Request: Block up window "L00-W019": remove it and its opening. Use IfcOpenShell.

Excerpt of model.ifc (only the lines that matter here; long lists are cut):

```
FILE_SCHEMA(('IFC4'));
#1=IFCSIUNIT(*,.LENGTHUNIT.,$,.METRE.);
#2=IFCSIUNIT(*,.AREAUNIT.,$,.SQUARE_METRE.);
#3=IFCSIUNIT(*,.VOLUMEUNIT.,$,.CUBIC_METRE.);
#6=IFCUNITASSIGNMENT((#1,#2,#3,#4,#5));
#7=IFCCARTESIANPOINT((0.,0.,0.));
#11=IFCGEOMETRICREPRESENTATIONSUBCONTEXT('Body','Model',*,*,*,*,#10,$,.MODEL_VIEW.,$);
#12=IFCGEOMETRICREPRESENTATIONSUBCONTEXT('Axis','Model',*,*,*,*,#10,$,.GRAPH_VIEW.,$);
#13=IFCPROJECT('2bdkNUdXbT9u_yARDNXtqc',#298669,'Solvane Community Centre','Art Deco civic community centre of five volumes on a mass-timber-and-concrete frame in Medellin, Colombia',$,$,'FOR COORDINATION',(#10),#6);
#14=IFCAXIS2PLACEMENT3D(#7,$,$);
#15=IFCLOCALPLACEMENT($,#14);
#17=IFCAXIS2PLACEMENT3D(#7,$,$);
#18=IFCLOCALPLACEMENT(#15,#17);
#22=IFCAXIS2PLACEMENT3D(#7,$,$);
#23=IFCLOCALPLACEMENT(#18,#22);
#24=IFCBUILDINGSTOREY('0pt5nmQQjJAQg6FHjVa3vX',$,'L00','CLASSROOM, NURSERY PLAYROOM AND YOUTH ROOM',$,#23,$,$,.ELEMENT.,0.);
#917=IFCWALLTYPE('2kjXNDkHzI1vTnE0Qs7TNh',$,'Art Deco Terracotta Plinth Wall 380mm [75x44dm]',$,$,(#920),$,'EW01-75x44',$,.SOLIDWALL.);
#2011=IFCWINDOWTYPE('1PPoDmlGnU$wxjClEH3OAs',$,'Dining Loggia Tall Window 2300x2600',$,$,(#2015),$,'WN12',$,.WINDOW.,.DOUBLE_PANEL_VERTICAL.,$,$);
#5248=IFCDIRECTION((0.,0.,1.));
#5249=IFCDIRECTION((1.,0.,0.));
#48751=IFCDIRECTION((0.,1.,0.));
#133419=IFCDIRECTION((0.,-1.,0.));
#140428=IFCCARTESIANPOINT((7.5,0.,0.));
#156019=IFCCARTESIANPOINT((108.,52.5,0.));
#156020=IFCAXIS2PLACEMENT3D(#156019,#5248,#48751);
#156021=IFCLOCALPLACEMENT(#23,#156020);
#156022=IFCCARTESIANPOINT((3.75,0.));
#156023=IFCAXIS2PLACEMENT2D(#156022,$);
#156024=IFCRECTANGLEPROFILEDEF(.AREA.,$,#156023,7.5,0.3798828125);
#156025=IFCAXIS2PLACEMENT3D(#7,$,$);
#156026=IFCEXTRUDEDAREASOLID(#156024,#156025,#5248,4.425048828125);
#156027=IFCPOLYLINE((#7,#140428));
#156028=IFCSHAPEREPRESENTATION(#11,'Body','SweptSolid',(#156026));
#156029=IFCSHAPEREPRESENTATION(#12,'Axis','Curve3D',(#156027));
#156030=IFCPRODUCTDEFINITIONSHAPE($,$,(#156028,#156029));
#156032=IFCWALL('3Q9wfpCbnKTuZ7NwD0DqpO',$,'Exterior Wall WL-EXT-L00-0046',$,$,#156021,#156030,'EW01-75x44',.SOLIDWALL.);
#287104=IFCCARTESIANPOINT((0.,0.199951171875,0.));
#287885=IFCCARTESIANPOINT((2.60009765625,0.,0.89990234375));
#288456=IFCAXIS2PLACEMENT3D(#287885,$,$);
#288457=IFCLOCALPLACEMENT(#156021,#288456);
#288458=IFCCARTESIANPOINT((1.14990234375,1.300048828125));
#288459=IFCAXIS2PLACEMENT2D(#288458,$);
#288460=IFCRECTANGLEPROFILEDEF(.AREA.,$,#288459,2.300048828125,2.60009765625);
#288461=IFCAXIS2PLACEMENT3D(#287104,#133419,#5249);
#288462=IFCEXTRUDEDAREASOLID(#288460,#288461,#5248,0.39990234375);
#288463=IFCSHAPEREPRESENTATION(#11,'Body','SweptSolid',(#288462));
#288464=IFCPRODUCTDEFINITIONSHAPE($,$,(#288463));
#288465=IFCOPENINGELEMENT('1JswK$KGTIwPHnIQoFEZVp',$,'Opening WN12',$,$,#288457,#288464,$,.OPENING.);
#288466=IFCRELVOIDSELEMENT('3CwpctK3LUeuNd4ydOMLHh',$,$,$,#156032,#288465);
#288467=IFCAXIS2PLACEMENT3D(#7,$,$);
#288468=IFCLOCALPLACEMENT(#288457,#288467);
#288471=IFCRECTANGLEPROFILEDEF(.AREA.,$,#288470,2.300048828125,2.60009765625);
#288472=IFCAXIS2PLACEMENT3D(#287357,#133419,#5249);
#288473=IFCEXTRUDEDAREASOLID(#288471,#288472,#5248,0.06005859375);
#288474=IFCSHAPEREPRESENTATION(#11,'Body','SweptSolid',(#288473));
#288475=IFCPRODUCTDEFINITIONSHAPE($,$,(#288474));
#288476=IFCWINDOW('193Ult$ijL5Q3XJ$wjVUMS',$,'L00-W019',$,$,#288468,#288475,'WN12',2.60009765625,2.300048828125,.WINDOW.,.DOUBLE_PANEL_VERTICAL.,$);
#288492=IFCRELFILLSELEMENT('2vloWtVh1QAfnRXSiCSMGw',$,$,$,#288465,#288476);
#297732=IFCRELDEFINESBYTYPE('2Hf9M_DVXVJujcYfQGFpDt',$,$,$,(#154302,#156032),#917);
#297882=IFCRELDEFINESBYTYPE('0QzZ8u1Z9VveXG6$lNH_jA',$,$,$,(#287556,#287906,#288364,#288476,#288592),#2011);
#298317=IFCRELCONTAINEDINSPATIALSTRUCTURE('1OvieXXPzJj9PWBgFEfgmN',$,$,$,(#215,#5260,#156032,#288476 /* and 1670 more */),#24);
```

```python
import ifcopenshell
import ifcopenshell.api.feature
import ifcopenshell.api.root
import ifcopenshell.geom
import ifcopenshell.util.shape

model = ifcopenshell.open("model.ifc")
settings = ifcopenshell.geom.settings()


def volume(element):
    """Net volume in cubic metres, openings subtracted."""
    shape = ifcopenshell.geom.create_shape(settings, element)
    return ifcopenshell.util.shape.get_volume(shape.geometry)


window = model.by_id(288476)
opening = window.FillsVoids[0].RelatingOpeningElement
wall = opening.VoidsElements[0].RelatingBuildingElement
before = volume(wall)

ifcopenshell.api.root.remove_product(model, product=window)
ifcopenshell.api.feature.remove_feature(model, feature=opening)

after = volume(wall)

print(f"wall volume {before:.3f} -> {after:.3f} m3")

model.write("model_updated.ifc")
```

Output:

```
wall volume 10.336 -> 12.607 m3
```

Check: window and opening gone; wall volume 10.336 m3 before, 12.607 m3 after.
